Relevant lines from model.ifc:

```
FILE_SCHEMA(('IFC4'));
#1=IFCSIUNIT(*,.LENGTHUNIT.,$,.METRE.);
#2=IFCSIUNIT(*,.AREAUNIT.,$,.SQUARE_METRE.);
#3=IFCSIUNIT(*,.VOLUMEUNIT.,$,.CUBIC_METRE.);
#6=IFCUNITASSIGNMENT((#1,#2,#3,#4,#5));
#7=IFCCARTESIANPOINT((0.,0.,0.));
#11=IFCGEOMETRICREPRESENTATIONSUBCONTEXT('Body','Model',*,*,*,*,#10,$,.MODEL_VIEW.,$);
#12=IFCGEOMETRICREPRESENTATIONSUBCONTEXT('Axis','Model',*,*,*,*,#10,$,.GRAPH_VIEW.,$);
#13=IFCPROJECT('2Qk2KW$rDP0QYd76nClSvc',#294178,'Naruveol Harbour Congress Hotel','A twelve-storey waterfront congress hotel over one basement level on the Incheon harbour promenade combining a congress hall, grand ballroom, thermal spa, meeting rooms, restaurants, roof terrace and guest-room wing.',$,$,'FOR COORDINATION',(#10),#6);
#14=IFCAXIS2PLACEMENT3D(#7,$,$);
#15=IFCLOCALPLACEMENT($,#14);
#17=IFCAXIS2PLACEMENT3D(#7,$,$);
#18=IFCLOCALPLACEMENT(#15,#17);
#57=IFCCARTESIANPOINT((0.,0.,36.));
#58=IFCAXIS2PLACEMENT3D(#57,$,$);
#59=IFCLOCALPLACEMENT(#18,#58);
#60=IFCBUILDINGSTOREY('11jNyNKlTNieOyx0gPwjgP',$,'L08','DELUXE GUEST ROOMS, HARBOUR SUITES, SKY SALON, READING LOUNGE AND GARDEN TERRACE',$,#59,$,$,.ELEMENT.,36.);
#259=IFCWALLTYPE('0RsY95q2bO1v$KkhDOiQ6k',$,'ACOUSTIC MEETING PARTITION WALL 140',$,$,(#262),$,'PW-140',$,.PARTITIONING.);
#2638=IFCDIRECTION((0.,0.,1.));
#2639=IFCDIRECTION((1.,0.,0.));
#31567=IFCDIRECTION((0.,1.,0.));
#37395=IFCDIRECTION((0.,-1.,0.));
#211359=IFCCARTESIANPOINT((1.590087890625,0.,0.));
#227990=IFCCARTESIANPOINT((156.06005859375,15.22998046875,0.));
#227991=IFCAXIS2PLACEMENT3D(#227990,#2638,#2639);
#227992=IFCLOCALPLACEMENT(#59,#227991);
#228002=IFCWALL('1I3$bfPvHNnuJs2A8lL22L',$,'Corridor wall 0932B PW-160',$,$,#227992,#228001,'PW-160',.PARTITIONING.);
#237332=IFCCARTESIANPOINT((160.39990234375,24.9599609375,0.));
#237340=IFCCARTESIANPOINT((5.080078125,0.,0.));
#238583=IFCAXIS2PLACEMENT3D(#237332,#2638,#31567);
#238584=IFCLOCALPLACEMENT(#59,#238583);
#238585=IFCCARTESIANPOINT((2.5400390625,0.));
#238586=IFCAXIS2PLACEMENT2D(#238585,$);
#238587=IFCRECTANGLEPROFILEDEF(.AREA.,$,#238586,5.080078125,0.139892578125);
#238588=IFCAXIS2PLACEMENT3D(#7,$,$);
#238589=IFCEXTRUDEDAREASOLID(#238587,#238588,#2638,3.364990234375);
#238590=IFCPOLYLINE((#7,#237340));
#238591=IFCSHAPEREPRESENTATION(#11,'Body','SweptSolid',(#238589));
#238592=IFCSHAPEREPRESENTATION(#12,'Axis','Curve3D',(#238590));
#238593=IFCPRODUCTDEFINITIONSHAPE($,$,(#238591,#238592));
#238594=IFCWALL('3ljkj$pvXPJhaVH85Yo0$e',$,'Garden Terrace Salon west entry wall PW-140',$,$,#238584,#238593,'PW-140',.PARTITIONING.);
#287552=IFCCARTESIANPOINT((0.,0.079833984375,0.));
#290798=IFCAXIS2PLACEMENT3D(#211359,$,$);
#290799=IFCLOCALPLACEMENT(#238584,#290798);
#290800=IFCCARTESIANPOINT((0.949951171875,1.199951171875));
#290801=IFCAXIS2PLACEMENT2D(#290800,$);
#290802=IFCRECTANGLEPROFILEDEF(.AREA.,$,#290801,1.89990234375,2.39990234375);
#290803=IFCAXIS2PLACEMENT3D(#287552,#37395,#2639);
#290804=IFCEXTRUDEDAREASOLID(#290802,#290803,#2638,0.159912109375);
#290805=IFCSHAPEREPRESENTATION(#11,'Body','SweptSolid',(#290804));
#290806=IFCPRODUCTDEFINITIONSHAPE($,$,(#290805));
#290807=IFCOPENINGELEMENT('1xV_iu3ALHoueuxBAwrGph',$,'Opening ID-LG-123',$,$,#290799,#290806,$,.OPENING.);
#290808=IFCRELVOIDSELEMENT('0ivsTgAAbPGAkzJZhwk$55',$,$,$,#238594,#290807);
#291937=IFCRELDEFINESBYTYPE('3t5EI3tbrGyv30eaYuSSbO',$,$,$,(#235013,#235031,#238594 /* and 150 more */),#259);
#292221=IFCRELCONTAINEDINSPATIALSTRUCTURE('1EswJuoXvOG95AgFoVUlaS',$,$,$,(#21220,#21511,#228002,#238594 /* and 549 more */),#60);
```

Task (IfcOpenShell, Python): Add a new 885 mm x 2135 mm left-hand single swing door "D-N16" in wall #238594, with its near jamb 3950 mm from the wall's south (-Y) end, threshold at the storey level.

```python
import numpy as np
import ifcopenshell
import ifcopenshell.api.feature
import ifcopenshell.api.geometry
import ifcopenshell.api.root
import ifcopenshell.api.spatial
import ifcopenshell.geom
import ifcopenshell.util.element
import ifcopenshell.util.placement
import ifcopenshell.util.representation
import ifcopenshell.util.shape
import ifcopenshell.util.unit

model = ifcopenshell.open("model.ifc")
unit_scale = ifcopenshell.util.unit.calculate_unit_scale(model)
settings = ifcopenshell.geom.settings()


def volume(element):
    """Net volume in cubic metres, openings subtracted."""
    shape = ifcopenshell.geom.create_shape(settings, element)
    return ifcopenshell.util.shape.get_volume(shape.geometry)


wall = model.by_guid("3ljkj$pvXPJhaVH85Yo0$e")
storey = ifcopenshell.util.element.get_container(wall, ifc_class="IfcBuildingStorey")
context = ifcopenshell.util.representation.get_context(model, "Model", "Body", "MODEL_VIEW")
before = volume(wall)

width, height, from_end, sill = 0.885, 2.135, 3.95, 0.0  # metres

# The wall runs along its own X axis, and the end named is its -X end.
wall_shape = ifcopenshell.geom.create_shape(settings, wall)
x, y, z = ifcopenshell.util.shape.get_vertices(wall_shape.geometry).T
start = x.min() + from_end
face, thickness = float(y.min()), float(y.max() - y.min())
wall_matrix = ifcopenshell.util.placement.get_local_placement(wall.ObjectPlacement)
level = ifcopenshell.util.placement.get_local_placement(storey.ObjectPlacement)[2, 3]


def in_wall(x, y):
    """Placement at x, y metres in the wall's axes, at sill height."""
    matrix = wall_matrix.copy()
    matrix[:, 3] = wall_matrix @ np.array([x / unit_scale, y / unit_scale, 0.0, 1.0])
    matrix[2, 3] = level + sill / unit_scale
    return matrix


# Opening: a box that overshoots both wall faces by 50 mm.
opening = ifcopenshell.api.root.create_entity(model, ifc_class="IfcOpeningElement", predefined_type="OPENING")
box = ifcopenshell.api.geometry.add_wall_representation(
    model, context=context, length=width, height=height, thickness=thickness + 0.1
)
ifcopenshell.api.geometry.assign_representation(model, product=opening, representation=box)
ifcopenshell.api.geometry.edit_object_placement(model, product=opening, matrix=in_wall(start, face - 0.05), is_si=False)
ifcopenshell.api.feature.add_feature(model, feature=opening, element=wall)

door = ifcopenshell.api.root.create_entity(model, ifc_class="IfcDoor", name="D-N16", predefined_type="DOOR")
door.OverallWidth, door.OverallHeight = width / unit_scale, height / unit_scale
door.OperationType = "SINGLE_SWING_LEFT"
body = ifcopenshell.api.geometry.add_door_representation(
    model,
    context=context,
    overall_width=door.OverallWidth,
    overall_height=door.OverallHeight,
    operation_type="SINGLE_SWING_LEFT",
    lining_properties={"LiningDepth": thickness / unit_scale, "ThresholdDepth": thickness / unit_scale},
)
ifcopenshell.api.geometry.assign_representation(model, product=door, representation=body)
ifcopenshell.api.spatial.assign_container(model, products=[door], relating_structure=storey)
ifcopenshell.api.feature.add_filling(model, opening=opening, element=door)

# The lining spans the wall, so the door starts at the wall face.
ifcopenshell.api.geometry.edit_object_placement(model, product=door, matrix=in_wall(start, face), is_si=False)

after = volume(wall)

print(f"wall volume {before:.3f} -> {after:.3f} m3")

model.write("model_updated.ifc")
```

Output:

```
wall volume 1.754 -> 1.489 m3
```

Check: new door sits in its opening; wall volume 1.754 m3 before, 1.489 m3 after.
